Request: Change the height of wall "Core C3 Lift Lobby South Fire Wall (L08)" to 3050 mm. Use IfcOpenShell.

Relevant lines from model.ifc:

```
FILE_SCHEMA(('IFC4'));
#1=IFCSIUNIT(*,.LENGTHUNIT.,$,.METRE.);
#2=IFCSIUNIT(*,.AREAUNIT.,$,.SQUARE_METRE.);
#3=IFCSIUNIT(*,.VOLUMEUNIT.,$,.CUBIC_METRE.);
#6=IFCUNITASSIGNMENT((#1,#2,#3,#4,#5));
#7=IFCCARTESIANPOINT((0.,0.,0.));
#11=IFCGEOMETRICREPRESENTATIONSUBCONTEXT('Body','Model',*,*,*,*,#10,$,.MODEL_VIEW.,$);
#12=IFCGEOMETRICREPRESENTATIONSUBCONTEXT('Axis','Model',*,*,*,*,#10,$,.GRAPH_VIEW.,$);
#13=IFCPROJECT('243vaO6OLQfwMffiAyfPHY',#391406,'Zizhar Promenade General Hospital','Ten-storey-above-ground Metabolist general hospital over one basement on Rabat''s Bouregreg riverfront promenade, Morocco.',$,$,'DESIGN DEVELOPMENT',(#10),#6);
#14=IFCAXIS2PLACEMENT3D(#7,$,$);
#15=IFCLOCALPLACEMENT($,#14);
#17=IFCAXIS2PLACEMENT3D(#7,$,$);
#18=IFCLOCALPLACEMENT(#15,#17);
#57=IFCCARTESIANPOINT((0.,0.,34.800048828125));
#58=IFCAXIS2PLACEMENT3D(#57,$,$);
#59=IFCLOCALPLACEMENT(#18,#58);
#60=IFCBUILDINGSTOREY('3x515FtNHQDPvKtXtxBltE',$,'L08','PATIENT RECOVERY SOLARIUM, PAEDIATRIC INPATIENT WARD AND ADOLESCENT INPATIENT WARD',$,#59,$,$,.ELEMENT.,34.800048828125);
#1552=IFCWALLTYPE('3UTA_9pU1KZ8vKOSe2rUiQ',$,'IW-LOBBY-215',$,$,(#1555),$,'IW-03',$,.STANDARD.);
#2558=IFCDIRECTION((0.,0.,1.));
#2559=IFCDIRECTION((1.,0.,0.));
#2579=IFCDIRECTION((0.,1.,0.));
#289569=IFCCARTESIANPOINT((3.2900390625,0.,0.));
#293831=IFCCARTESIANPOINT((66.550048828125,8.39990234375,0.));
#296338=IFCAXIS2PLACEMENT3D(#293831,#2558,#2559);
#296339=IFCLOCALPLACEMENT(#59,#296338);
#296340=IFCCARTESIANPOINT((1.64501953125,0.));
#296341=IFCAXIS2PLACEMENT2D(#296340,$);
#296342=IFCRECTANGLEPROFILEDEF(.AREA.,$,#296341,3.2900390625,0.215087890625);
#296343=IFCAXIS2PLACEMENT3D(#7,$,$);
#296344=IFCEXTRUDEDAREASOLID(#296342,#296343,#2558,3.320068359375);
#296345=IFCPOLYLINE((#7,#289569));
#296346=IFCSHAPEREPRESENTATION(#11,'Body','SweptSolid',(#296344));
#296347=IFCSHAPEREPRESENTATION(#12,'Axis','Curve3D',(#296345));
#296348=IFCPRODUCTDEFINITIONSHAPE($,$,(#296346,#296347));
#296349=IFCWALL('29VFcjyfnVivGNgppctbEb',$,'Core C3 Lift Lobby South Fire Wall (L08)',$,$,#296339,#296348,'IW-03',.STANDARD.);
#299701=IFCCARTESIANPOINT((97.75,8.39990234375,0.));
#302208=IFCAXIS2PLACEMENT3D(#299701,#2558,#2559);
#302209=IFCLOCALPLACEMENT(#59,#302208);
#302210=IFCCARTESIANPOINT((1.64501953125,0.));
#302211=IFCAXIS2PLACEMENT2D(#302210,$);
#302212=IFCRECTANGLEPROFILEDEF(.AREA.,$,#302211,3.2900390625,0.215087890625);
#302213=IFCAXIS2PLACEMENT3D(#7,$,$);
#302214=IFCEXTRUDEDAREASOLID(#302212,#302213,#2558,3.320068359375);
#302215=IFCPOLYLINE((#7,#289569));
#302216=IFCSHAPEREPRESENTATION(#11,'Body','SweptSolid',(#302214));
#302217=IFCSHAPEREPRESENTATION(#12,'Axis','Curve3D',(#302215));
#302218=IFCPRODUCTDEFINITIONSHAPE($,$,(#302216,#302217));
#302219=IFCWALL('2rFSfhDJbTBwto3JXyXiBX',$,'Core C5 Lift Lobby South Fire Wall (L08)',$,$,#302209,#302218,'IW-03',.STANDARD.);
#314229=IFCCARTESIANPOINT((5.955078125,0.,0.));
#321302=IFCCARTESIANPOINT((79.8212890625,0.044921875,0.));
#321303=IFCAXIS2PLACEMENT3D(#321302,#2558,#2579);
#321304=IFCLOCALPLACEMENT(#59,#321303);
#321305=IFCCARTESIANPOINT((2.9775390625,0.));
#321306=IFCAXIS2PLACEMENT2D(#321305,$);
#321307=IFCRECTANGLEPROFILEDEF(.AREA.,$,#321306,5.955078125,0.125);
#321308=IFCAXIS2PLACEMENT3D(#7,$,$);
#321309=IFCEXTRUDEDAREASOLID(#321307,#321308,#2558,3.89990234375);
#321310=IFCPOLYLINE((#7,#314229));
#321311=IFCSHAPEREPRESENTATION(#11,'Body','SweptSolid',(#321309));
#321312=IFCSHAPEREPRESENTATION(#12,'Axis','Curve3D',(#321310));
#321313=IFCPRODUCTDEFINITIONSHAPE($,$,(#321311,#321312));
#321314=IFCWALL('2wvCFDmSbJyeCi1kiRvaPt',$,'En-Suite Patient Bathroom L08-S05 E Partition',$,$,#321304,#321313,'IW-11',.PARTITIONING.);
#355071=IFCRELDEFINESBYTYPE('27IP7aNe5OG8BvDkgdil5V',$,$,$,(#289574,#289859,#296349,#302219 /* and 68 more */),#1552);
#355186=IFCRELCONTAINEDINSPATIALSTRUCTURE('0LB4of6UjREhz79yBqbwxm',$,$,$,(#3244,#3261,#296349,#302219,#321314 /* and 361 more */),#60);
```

```python
import ifcopenshell
import ifcopenshell.geom
import ifcopenshell.util.representation
import ifcopenshell.util.shape

model = ifcopenshell.open("model.ifc")
settings = ifcopenshell.geom.settings()


def volume(element):
    """Net volume in cubic metres, openings subtracted."""
    shape = ifcopenshell.geom.create_shape(settings, element)
    return ifcopenshell.util.shape.get_volume(shape.geometry)


wall = model.by_guid("29VFcjyfnVivGNgppctbEb")
before = volume(wall)

body = ifcopenshell.util.representation.get_representation(wall, "Model", "Body")
solid = body.Items[0]
old_height = solid.Depth
solid.Depth = 3.05
after = volume(wall)

print(f"height {old_height:g} -> {solid.Depth:g}, volume {before:.3f} -> {after:.3f} m3")

model.write("model_rev.ifc")
```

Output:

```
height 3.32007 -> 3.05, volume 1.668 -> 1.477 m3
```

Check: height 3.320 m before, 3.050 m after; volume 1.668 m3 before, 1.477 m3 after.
